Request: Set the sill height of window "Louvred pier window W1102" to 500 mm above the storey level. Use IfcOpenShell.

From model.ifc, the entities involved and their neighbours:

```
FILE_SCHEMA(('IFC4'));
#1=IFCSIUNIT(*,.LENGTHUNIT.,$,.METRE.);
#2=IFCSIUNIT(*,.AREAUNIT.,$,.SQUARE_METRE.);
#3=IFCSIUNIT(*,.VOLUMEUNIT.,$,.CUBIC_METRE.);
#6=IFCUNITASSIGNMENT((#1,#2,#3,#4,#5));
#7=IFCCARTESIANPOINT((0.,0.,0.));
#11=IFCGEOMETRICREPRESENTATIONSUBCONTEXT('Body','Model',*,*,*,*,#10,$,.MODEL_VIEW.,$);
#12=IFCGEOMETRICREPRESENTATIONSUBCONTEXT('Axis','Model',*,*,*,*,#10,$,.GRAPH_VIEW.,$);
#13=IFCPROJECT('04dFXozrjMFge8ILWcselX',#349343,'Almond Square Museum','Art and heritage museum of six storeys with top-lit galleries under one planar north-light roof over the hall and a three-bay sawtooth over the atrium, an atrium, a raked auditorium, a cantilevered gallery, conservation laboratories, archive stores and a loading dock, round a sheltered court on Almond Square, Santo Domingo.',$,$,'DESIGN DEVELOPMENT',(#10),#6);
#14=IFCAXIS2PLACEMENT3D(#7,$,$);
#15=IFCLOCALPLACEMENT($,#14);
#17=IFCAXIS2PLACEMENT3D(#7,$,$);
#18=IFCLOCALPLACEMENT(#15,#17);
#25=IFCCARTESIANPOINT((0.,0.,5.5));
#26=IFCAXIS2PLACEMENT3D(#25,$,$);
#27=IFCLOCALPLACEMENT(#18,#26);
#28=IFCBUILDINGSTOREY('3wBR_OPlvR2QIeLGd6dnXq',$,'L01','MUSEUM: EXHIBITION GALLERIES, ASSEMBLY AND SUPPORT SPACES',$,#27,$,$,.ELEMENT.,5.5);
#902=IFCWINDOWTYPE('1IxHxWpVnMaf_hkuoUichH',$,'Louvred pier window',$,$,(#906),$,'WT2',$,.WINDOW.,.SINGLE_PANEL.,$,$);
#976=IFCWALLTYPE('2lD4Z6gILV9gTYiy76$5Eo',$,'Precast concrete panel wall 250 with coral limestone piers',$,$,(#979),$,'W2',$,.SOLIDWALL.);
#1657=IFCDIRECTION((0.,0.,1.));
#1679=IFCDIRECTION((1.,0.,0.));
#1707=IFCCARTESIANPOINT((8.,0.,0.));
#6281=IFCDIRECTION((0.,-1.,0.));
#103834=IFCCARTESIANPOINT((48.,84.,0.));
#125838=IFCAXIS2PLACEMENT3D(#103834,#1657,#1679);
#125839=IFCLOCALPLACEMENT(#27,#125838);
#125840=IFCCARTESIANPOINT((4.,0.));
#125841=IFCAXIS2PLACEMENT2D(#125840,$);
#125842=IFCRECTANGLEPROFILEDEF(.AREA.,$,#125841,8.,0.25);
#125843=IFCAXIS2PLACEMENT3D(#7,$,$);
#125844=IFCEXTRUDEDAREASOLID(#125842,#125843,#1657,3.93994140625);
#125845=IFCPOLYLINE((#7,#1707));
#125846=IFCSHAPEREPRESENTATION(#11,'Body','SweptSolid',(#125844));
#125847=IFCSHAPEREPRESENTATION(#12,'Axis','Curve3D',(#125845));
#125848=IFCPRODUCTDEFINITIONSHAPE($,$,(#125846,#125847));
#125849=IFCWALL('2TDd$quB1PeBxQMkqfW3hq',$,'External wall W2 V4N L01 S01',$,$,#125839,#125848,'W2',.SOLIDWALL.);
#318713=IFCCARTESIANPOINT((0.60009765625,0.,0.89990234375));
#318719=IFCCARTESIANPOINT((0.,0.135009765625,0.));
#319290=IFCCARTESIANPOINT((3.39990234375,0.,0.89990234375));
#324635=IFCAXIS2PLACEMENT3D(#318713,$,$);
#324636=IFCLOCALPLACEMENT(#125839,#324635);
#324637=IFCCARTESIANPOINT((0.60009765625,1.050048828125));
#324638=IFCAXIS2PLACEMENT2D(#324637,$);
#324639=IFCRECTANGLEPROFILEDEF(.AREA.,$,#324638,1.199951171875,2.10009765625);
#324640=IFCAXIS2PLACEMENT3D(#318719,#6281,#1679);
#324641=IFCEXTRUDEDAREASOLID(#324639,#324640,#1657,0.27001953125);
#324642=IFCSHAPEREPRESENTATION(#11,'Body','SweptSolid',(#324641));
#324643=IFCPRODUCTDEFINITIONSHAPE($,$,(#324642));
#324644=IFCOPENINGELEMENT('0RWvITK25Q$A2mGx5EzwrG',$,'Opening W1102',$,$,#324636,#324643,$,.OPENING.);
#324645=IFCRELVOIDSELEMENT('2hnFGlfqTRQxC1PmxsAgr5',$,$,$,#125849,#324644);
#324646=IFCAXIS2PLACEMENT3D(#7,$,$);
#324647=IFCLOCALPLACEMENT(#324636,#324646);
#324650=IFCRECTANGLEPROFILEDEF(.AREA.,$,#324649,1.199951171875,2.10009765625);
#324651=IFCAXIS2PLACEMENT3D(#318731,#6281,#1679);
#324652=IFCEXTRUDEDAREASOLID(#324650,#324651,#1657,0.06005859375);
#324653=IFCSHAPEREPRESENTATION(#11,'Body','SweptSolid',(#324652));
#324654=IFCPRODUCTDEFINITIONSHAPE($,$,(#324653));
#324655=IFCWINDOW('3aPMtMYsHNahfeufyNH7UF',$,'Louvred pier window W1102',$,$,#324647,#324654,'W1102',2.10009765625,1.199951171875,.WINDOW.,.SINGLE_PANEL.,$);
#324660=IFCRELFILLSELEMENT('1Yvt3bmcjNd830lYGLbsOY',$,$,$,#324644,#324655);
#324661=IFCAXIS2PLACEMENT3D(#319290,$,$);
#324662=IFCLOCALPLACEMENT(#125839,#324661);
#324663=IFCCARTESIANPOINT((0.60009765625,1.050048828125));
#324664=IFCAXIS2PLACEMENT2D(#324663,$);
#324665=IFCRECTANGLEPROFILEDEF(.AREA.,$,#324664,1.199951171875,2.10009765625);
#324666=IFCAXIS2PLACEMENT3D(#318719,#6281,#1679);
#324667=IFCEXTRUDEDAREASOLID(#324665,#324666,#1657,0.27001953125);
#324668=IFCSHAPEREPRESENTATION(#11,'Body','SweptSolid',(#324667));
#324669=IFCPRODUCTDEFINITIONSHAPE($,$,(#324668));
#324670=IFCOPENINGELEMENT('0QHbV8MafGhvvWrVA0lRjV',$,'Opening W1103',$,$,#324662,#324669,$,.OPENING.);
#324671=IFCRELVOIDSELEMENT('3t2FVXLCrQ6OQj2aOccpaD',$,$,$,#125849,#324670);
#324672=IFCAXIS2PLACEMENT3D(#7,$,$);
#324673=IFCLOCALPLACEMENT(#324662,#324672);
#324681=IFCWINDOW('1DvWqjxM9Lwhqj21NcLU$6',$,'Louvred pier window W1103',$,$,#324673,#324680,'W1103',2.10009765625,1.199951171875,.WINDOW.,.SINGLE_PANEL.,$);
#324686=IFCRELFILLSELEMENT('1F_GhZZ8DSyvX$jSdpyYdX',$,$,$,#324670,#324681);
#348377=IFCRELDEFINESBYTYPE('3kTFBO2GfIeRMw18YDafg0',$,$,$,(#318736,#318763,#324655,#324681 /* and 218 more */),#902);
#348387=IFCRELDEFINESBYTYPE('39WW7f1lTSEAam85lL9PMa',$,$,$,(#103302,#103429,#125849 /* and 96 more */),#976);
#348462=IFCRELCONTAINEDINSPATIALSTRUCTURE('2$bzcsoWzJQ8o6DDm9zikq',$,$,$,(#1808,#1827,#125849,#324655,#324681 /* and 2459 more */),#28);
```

```python
import numpy as np
import ifcopenshell
import ifcopenshell.api.geometry
import ifcopenshell.geom
import ifcopenshell.util.element
import ifcopenshell.util.placement
import ifcopenshell.util.shape
import ifcopenshell.util.unit

model = ifcopenshell.open("model.ifc")
unit_scale = ifcopenshell.util.unit.calculate_unit_scale(model)

window = model.by_guid("3aPMtMYsHNahfeufyNH7UF")
opening = window.FillsVoids[0].RelatingOpeningElement
storey = ifcopenshell.util.element.get_container(window, ifc_class="IfcBuildingStorey")
level = ifcopenshell.util.placement.get_local_placement(storey.ObjectPlacement)[2, 3]

# The opening's origin need not be at the sill, so measure its lowest point.
shape = ifcopenshell.geom.create_shape(ifcopenshell.geom.settings(), opening)
bottom = ifcopenshell.util.shape.get_shape_bottom_elevation(shape, shape.geometry) / unit_scale
dz = level + 0.5 - bottom

shift = np.array([0.0, 0.0, dz])
# The window is placed relative to its opening, so it follows when the opening moves.
matrix = ifcopenshell.util.placement.get_local_placement(opening.ObjectPlacement)
matrix[:3, 3] += shift
ifcopenshell.api.geometry.edit_object_placement(
    model, product=opening, matrix=matrix, is_si=False, should_transform_children=True
)

print(f"moved by {dz * unit_scale:+.3f} m")

model.write("model-out.ifc")
```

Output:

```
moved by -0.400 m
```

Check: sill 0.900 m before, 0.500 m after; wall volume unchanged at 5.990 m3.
